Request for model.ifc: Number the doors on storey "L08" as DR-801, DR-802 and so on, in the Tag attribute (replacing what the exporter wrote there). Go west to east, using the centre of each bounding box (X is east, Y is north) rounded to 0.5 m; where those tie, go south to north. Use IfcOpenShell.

First a look at what the model holds.

```python
import ifcopenshell
import ifcopenshell.util.element
import ifcopenshell.util.placement

model = ifcopenshell.open("model.ifc")
print(model.schema)
storey = next(s for s in model.by_type("IfcBuildingStorey") if s.Name == "L08")
doors = [e for e in ifcopenshell.util.element.get_decomposition(storey) if e.is_a("IfcDoor")]
for e in sorted(doors, key=lambda e: e.id()):
    origin = ifcopenshell.util.placement.get_local_placement(e.ObjectPlacement)[:3, 3]
    print(e.id(), e.Tag, e.Name, origin.round(2) + 0.0, sep=" | ")
```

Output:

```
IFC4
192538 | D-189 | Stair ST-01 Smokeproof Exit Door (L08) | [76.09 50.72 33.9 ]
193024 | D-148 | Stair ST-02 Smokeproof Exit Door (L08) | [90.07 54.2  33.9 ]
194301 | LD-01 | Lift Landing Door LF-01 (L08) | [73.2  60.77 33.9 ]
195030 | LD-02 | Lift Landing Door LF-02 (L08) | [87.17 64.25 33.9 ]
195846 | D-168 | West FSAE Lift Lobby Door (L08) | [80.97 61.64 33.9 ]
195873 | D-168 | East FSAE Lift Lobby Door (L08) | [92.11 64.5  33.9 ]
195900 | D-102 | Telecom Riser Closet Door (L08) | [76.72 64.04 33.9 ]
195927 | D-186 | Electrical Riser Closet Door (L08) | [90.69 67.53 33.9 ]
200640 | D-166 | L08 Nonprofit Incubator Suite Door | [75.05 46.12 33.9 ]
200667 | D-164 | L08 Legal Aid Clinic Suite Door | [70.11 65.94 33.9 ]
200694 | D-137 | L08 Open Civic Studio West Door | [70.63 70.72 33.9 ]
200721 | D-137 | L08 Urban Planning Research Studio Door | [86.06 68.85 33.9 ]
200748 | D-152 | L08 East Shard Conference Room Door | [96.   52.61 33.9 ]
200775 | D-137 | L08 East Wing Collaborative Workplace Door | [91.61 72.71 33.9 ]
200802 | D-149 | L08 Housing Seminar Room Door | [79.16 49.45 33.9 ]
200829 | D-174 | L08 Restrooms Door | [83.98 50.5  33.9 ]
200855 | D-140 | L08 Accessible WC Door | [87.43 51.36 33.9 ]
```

```python
import ifcopenshell
import ifcopenshell.geom
import ifcopenshell.util.element
import ifcopenshell.util.shape

model = ifcopenshell.open("model.ifc")
settings = ifcopenshell.geom.settings()
settings.set("use-world-coords", True)


def centre(element):
    shape = ifcopenshell.geom.create_shape(settings, element)
    return ifcopenshell.util.shape.get_bbox_centroid(shape.geometry)


storey = next(s for s in model.by_type("IfcBuildingStorey") if s.Name == "L08")
doors = [e for e in ifcopenshell.util.element.get_decomposition(storey) if e.is_a("IfcDoor")]

# Insertion points can sit at a corner or the storey origin, so sort by the geometry (in metres).
centres = {e: centre(e) for e in doors}
doors.sort(key=lambda e: (round(centres[e][0] / 0.5), centres[e][1]))

for i, e in enumerate(doors, start=1):
    number = f"DR-8{i:02d}"
    e.Tag = number
    print(e.id(), number)

model.write("model_rev.ifc")
```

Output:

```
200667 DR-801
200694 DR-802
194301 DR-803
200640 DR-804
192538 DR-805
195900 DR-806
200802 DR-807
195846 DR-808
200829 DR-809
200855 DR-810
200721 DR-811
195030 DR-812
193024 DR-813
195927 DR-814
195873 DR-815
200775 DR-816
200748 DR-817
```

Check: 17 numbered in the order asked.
